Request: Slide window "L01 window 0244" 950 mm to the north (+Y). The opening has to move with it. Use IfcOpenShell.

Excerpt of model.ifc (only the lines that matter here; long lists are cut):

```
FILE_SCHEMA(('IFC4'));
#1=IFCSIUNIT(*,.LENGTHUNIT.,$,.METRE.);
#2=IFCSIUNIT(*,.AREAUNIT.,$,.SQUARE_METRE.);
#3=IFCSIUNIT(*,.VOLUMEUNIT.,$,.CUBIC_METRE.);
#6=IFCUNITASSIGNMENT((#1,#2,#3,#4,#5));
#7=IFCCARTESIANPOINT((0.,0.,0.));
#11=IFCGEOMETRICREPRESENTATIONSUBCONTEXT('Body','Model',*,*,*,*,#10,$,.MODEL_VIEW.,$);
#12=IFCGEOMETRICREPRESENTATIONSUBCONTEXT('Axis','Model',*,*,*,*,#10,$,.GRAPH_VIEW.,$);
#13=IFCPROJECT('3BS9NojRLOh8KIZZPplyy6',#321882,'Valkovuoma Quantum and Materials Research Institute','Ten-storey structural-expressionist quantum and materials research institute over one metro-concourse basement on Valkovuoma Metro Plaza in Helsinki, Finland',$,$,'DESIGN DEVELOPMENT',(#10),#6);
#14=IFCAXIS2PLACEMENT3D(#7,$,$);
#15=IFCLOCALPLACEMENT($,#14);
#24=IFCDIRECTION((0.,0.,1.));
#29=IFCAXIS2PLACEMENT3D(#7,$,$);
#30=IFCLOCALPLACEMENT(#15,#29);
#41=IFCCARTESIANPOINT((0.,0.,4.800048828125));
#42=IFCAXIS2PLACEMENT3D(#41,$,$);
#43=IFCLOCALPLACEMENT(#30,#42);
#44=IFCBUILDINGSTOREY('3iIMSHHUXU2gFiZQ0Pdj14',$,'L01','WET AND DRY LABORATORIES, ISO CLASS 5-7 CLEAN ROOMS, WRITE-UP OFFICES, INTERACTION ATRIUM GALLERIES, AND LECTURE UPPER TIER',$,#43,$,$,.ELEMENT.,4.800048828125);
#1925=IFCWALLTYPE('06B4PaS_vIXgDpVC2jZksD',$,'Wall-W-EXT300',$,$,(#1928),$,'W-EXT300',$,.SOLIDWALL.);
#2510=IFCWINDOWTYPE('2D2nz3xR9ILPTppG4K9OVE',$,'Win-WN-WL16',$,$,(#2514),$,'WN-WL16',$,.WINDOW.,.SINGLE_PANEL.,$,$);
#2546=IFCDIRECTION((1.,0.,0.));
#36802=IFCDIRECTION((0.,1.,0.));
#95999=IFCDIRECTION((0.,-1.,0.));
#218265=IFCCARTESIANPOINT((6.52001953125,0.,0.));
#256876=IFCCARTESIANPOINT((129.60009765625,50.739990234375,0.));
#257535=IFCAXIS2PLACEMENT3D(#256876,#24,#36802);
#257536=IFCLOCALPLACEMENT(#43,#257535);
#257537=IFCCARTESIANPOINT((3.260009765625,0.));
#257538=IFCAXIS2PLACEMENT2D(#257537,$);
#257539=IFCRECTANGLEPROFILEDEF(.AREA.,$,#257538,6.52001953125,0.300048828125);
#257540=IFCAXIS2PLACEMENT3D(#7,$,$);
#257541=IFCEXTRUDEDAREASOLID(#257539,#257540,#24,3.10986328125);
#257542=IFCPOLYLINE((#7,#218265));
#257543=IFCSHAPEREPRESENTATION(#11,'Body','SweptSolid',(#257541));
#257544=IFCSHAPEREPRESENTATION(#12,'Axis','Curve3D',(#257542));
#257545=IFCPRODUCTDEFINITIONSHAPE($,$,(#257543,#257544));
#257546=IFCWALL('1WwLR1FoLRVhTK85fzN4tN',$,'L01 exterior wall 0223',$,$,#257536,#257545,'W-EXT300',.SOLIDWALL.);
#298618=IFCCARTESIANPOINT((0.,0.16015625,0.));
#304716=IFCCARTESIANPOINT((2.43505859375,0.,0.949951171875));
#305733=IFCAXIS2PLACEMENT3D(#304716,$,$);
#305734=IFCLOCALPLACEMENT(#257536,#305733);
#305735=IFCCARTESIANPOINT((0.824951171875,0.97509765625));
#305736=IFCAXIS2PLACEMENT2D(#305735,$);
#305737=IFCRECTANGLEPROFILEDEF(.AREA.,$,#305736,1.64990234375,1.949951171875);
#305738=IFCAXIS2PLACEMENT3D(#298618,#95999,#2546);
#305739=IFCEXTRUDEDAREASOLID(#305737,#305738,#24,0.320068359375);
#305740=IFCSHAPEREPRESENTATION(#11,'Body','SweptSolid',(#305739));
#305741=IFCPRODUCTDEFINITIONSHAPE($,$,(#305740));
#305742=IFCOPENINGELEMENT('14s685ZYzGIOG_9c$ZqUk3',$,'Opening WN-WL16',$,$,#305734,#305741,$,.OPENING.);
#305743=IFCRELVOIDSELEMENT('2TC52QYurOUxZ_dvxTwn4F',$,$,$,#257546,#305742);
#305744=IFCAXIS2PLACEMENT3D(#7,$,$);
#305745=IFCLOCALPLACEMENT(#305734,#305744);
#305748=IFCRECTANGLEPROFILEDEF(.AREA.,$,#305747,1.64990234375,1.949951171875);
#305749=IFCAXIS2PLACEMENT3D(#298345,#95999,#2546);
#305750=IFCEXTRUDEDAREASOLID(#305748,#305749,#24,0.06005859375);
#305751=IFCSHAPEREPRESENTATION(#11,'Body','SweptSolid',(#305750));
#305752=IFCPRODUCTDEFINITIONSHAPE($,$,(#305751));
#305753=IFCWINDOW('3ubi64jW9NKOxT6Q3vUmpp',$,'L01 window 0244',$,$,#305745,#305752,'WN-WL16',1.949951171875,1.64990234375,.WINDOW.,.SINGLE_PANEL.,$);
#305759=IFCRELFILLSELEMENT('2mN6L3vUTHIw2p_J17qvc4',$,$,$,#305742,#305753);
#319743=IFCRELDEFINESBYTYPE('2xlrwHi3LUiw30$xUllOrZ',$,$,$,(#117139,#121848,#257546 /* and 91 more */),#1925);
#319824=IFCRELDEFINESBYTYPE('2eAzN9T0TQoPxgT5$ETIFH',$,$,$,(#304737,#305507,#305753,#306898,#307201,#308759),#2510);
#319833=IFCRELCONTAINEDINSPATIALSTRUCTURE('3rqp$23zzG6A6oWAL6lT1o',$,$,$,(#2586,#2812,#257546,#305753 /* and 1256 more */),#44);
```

```python
import ifcopenshell
import ifcopenshell.api.geometry
import ifcopenshell.util.placement
import ifcopenshell.util.unit

model = ifcopenshell.open("model.ifc")
unit_scale = ifcopenshell.util.unit.calculate_unit_scale(model)

window = model.by_guid("3ubi64jW9NKOxT6Q3vUmpp")
opening = window.FillsVoids[0].RelatingOpeningElement
wall = opening.VoidsElements[0].RelatingBuildingElement

wall_matrix = ifcopenshell.util.placement.get_local_placement(wall.ObjectPlacement)
shift = wall_matrix[:3, 0] * 0.95 / unit_scale
before = ifcopenshell.util.placement.get_local_placement(window.ObjectPlacement)[:3, 3].copy()

# The window is placed relative to its opening, so it follows when the opening moves.
matrix = ifcopenshell.util.placement.get_local_placement(opening.ObjectPlacement)
matrix[:3, 3] += shift
ifcopenshell.api.geometry.edit_object_placement(
    model, product=opening, matrix=matrix, is_si=False, should_transform_children=True
)

after = ifcopenshell.util.placement.get_local_placement(window.ObjectPlacement)[:3, 3]
print("window moved by", (after - before).round(3) + 0.0)

model.write("model_updated.ifc")
```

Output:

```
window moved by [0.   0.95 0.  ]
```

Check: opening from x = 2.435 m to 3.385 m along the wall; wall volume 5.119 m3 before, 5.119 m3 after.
